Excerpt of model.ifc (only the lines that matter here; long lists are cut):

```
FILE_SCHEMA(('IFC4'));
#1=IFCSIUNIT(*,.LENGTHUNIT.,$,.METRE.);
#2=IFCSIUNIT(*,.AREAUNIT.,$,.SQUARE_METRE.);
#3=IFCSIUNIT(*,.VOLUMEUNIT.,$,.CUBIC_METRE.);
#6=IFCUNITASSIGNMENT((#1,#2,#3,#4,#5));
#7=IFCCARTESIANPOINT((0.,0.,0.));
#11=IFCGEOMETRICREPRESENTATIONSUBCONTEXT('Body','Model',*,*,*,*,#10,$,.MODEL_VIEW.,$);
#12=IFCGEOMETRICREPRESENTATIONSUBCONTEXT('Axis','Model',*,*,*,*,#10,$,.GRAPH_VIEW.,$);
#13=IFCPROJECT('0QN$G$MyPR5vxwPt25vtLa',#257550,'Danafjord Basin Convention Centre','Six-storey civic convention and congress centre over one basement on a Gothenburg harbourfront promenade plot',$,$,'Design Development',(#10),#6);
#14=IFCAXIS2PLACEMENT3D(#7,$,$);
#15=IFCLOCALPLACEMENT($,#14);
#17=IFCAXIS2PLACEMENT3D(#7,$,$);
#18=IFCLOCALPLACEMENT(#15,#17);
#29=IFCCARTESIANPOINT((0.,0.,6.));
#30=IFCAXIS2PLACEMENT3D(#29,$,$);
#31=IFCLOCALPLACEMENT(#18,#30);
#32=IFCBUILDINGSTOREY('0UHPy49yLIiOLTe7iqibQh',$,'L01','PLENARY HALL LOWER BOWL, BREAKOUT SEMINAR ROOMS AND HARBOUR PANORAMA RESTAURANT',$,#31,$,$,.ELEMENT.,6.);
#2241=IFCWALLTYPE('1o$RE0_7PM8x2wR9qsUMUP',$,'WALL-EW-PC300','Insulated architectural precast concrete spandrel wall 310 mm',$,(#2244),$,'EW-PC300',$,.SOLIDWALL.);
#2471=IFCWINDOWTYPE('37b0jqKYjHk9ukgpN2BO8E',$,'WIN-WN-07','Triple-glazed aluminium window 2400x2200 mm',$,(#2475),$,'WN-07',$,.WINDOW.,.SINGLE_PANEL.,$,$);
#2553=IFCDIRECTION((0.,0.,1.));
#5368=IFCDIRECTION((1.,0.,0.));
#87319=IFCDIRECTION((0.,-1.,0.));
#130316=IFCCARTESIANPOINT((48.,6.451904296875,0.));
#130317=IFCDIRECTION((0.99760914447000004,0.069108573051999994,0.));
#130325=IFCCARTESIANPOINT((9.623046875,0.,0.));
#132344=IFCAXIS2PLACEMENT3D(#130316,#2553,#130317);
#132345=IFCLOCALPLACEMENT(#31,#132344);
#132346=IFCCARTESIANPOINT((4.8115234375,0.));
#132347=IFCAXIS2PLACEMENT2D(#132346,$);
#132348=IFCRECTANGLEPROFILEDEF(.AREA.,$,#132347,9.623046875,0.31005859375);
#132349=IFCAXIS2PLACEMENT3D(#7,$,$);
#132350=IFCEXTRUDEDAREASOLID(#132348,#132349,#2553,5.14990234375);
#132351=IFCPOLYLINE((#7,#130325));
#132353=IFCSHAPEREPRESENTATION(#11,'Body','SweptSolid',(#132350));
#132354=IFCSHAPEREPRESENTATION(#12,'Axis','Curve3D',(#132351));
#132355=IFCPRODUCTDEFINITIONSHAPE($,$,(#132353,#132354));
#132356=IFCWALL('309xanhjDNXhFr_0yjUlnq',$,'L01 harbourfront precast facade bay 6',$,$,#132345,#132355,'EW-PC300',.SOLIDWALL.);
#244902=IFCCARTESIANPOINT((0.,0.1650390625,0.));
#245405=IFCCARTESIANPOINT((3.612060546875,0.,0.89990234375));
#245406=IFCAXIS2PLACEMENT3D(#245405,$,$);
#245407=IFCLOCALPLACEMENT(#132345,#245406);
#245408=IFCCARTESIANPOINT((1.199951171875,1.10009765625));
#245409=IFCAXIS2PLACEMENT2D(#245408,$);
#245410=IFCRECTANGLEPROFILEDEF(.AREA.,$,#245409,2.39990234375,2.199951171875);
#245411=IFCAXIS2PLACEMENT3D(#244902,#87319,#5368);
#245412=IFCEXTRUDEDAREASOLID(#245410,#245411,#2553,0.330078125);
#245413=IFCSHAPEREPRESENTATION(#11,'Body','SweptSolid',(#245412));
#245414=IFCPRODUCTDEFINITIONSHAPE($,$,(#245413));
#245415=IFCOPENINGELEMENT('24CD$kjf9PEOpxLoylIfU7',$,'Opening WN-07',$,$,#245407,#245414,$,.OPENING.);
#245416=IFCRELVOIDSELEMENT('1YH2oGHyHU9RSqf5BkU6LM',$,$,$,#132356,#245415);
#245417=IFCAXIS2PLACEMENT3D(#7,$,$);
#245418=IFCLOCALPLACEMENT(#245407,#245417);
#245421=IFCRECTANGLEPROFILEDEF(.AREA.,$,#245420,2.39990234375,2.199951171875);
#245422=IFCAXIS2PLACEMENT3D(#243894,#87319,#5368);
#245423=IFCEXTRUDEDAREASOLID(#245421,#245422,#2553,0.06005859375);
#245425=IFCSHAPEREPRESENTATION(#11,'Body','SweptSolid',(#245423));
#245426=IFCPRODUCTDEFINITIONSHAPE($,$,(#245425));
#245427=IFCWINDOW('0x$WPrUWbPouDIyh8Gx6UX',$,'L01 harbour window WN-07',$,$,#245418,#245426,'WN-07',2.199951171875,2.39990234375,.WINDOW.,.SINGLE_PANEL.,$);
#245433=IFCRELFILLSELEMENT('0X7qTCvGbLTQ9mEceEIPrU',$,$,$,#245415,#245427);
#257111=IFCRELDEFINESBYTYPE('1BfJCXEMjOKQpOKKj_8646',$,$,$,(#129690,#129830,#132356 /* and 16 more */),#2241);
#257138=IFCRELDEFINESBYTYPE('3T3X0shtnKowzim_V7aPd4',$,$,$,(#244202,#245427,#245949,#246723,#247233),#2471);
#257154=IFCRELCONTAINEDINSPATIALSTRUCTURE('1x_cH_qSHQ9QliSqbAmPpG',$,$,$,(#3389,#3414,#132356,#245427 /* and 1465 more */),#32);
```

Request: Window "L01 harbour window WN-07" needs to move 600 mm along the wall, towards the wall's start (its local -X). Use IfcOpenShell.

```python
import ifcopenshell
import ifcopenshell.api.geometry
import ifcopenshell.util.placement
import ifcopenshell.util.unit

model = ifcopenshell.open("model.ifc")
unit_scale = ifcopenshell.util.unit.calculate_unit_scale(model)

window = model.by_guid("0x$WPrUWbPouDIyh8Gx6UX")
opening = window.FillsVoids[0].RelatingOpeningElement
wall = opening.VoidsElements[0].RelatingBuildingElement

wall_matrix = ifcopenshell.util.placement.get_local_placement(wall.ObjectPlacement)
shift = wall_matrix[:3, 0] * -0.6 / unit_scale
before = ifcopenshell.util.placement.get_local_placement(window.ObjectPlacement)[:3, 3].copy()

# The window is placed relative to its opening, so it follows when the opening moves.
matrix = ifcopenshell.util.placement.get_local_placement(opening.ObjectPlacement)
matrix[:3, 3] += shift
ifcopenshell.api.geometry.edit_object_placement(
    model, product=opening, matrix=matrix, is_si=False, should_transform_children=True
)

after = ifcopenshell.util.placement.get_local_placement(window.ObjectPlacement)[:3, 3]
print("window moved by", (after - before).round(3) + 0.0)

model.write("model_updated.ifc")
```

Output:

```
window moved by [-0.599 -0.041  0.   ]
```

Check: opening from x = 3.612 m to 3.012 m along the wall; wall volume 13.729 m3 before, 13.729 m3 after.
